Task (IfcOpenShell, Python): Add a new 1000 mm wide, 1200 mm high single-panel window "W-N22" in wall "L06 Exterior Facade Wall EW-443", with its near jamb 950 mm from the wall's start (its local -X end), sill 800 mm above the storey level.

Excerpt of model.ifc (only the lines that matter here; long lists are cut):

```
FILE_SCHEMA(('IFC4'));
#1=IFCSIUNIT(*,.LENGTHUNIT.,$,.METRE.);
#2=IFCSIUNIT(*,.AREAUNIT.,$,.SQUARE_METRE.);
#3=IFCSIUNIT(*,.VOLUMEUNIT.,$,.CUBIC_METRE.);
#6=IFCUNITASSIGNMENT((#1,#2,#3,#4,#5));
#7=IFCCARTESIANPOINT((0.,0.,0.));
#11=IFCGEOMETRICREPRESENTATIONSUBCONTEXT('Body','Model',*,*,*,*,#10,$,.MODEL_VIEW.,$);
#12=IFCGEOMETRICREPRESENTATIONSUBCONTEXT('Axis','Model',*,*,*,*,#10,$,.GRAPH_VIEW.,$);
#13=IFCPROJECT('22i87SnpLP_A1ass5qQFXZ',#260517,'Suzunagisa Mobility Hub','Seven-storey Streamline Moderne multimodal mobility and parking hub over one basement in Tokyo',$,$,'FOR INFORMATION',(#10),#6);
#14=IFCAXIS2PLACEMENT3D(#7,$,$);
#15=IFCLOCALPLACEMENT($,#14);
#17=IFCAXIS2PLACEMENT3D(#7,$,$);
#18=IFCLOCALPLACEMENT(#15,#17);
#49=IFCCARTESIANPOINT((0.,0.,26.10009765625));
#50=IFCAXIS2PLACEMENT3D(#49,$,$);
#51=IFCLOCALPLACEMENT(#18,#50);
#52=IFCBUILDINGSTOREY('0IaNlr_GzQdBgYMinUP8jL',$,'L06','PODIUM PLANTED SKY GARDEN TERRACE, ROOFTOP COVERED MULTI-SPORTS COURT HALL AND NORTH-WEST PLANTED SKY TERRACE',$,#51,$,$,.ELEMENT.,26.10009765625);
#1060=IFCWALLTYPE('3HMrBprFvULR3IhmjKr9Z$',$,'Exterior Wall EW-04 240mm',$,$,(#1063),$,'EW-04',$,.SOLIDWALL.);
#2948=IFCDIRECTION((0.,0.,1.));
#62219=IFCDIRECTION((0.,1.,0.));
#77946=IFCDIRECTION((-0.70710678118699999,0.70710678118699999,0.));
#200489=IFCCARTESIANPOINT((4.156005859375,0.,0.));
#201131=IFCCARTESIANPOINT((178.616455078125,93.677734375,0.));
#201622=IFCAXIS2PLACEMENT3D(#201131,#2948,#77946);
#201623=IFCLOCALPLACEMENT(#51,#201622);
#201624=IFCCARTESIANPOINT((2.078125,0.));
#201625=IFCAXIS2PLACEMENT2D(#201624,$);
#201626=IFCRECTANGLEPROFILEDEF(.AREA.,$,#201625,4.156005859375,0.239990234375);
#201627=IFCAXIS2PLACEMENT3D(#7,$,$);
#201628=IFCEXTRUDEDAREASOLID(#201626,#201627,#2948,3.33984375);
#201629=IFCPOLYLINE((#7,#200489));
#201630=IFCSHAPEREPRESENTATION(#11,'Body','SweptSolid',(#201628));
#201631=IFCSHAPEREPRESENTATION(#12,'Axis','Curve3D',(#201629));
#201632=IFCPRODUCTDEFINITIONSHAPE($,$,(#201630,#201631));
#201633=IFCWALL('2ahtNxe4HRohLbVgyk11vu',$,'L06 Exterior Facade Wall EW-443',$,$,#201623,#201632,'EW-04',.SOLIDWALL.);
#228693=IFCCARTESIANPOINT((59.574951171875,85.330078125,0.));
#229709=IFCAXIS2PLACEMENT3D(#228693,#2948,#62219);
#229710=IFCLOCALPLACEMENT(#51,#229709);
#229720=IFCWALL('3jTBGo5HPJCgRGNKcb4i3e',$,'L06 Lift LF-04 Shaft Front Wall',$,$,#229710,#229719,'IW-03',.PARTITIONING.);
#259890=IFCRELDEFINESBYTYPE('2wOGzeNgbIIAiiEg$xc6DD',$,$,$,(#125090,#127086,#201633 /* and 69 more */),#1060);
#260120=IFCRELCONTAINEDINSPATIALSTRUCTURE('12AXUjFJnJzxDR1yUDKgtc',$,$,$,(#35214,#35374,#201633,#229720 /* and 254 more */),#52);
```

```python
import numpy as np
import ifcopenshell
import ifcopenshell.api.feature
import ifcopenshell.api.geometry
import ifcopenshell.api.root
import ifcopenshell.api.spatial
import ifcopenshell.geom
import ifcopenshell.util.element
import ifcopenshell.util.placement
import ifcopenshell.util.representation
import ifcopenshell.util.shape
import ifcopenshell.util.unit

model = ifcopenshell.open("model.ifc")
unit_scale = ifcopenshell.util.unit.calculate_unit_scale(model)
settings = ifcopenshell.geom.settings()


def volume(element):
    """Net volume in cubic metres, openings subtracted."""
    shape = ifcopenshell.geom.create_shape(settings, element)
    return ifcopenshell.util.shape.get_volume(shape.geometry)


wall = model.by_id(201633)
storey = ifcopenshell.util.element.get_container(wall, ifc_class="IfcBuildingStorey")
context = ifcopenshell.util.representation.get_context(model, "Model", "Body", "MODEL_VIEW")
before = volume(wall)

width, height, from_end, sill = 1, 1.2, 0.95, 0.8  # metres

# The wall runs along its own X axis, and the end named is its -X end.
wall_shape = ifcopenshell.geom.create_shape(settings, wall)
x, y, z = ifcopenshell.util.shape.get_vertices(wall_shape.geometry).T
start = x.min() + from_end
face, thickness = float(y.min()), float(y.max() - y.min())
wall_matrix = ifcopenshell.util.placement.get_local_placement(wall.ObjectPlacement)
level = ifcopenshell.util.placement.get_local_placement(storey.ObjectPlacement)[2, 3]


def in_wall(x, y):
    """Placement at x, y metres in the wall's axes, at sill height."""
    matrix = wall_matrix.copy()
    matrix[:, 3] = wall_matrix @ np.array([x / unit_scale, y / unit_scale, 0.0, 1.0])
    matrix[2, 3] = level + sill / unit_scale
    return matrix


# Opening: a box that overshoots both wall faces by 50 mm.
opening = ifcopenshell.api.root.create_entity(model, ifc_class="IfcOpeningElement", predefined_type="OPENING")
box = ifcopenshell.api.geometry.add_wall_representation(
    model, context=context, length=width, height=height, thickness=thickness + 0.1
)
ifcopenshell.api.geometry.assign_representation(model, product=opening, representation=box)
ifcopenshell.api.geometry.edit_object_placement(model, product=opening, matrix=in_wall(start, face - 0.05), is_si=False)
ifcopenshell.api.feature.add_feature(model, feature=opening, element=wall)

window = ifcopenshell.api.root.create_entity(model, ifc_class="IfcWindow", name="W-N22", predefined_type="WINDOW")
window.OverallWidth, window.OverallHeight = width / unit_scale, height / unit_scale
window.PartitioningType = "SINGLE_PANEL"
body = ifcopenshell.api.geometry.add_window_representation(
    model,
    context=context,
    overall_width=window.OverallWidth,
    overall_height=window.OverallHeight,
    partition_type="SINGLE_PANEL",
)
ifcopenshell.api.geometry.assign_representation(model, product=window, representation=body)
ifcopenshell.api.spatial.assign_container(model, products=[window], relating_structure=storey)
ifcopenshell.api.feature.add_filling(model, opening=opening, element=window)

# Centre the window in the wall's thickness.
ifcopenshell.api.geometry.edit_object_placement(model, product=window, matrix=in_wall(start, face), is_si=False)
window_shape = ifcopenshell.geom.create_shape(settings, window)
depth = ifcopenshell.util.shape.get_vertices(window_shape.geometry)[:, 1]
offset = face + thickness / 2 - (depth.min() + depth.max()) / 2
ifcopenshell.api.geometry.edit_object_placement(model, product=window, matrix=in_wall(start, offset), is_si=False)

after = volume(wall)

print(f"wall volume {before:.3f} -> {after:.3f} m3")

model.write("model-out.ifc")
```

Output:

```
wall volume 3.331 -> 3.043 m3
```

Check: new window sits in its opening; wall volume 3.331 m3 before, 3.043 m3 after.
